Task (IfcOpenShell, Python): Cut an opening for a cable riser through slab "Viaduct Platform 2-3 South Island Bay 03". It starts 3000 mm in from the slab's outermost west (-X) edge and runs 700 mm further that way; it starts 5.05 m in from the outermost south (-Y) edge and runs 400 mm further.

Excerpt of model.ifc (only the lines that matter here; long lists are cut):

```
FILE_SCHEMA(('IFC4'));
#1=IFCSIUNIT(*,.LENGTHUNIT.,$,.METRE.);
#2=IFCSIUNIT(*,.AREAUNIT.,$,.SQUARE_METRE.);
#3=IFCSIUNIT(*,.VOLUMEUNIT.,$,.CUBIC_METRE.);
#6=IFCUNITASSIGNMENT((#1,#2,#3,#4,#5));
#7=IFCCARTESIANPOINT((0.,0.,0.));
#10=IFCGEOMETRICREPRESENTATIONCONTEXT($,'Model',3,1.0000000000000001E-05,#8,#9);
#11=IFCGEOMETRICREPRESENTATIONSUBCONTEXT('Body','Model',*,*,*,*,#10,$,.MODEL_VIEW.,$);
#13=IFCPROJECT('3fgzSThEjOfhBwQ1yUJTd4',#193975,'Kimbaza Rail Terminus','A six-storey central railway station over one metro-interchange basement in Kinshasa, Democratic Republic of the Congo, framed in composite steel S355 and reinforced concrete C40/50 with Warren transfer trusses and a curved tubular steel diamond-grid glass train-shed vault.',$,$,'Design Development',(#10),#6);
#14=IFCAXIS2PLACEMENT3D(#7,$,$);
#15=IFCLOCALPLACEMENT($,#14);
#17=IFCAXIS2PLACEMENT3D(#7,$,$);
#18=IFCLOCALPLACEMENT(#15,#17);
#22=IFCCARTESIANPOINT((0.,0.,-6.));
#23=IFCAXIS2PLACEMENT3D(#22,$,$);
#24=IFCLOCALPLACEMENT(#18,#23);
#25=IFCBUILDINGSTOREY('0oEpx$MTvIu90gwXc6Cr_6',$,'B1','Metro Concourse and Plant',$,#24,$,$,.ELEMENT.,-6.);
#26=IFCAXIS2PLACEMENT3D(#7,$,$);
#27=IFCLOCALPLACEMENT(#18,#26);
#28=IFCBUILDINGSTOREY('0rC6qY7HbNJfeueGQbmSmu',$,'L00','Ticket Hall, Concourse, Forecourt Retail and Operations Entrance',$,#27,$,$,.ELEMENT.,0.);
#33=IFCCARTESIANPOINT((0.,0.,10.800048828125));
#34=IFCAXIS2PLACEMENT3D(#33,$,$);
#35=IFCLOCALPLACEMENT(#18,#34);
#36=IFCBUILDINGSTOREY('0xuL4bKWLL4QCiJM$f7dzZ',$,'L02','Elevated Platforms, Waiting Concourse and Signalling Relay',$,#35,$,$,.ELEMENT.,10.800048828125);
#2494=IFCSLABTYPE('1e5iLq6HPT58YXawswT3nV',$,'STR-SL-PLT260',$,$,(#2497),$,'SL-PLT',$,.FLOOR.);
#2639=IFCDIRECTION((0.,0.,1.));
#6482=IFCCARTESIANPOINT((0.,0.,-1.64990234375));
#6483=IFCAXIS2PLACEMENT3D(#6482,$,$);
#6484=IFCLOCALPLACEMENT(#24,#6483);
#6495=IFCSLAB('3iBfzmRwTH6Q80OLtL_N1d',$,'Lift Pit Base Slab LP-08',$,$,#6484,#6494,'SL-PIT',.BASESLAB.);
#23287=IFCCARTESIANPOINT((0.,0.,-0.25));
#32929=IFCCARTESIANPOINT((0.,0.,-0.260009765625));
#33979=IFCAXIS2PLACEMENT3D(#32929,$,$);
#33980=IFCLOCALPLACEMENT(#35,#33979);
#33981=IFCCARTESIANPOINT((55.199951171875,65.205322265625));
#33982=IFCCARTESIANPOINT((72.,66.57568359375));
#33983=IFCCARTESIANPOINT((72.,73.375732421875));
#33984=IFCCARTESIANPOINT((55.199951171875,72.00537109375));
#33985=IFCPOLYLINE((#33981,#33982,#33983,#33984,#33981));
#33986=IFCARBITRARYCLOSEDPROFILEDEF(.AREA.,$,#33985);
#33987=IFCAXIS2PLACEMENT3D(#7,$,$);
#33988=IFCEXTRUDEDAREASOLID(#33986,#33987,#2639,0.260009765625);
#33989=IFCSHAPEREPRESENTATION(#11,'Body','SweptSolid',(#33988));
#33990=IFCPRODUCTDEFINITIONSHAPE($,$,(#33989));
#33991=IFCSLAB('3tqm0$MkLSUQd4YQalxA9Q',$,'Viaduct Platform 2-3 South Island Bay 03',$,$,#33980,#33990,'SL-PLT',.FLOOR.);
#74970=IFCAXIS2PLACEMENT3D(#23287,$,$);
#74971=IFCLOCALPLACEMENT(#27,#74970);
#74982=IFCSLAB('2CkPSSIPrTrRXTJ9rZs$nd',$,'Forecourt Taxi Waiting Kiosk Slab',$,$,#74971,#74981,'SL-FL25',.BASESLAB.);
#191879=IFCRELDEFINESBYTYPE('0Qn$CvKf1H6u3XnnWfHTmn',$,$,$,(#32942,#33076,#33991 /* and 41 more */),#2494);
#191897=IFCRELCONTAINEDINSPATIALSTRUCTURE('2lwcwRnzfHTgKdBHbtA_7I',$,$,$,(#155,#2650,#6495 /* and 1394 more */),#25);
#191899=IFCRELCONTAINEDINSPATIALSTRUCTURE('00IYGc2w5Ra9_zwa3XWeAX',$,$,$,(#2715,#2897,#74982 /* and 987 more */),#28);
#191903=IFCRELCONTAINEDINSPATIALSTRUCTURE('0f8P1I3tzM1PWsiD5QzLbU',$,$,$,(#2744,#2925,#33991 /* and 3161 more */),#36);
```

```python
import numpy as np
import ifcopenshell
import ifcopenshell.api.feature
import ifcopenshell.api.geometry
import ifcopenshell.api.root
import ifcopenshell.geom
import ifcopenshell.util.placement
import ifcopenshell.util.representation
import ifcopenshell.util.shape
import ifcopenshell.util.unit

model = ifcopenshell.open("model.ifc")
unit_scale = ifcopenshell.util.unit.calculate_unit_scale(model)
settings = ifcopenshell.geom.settings()


def volume(element):
    """Net volume in cubic metres, openings subtracted."""
    shape = ifcopenshell.geom.create_shape(settings, element)
    return ifcopenshell.util.shape.get_volume(shape.geometry)


slab = model.by_guid("3tqm0$MkLSUQd4YQalxA9Q")
before = volume(slab)

# Extent in the slab's own axes, in metres. The edges named are its -X and -Y sides.
slab_shape = ifcopenshell.geom.create_shape(settings, slab)
vertices = ifcopenshell.util.shape.get_vertices(slab_shape.geometry)
x_min, y_min, bottom = vertices.min(axis=0)
top = vertices[:, 2].max()

opening = ifcopenshell.api.root.create_entity(model, ifc_class="IfcOpeningElement", name="Cable riser opening", predefined_type="OPENING")
context = ifcopenshell.util.representation.get_context(model, "Model", "Body", "MODEL_VIEW")
width, depth = 0.7, 0.4
outline = [(0.0, 0.0), (width, 0.0), (width, depth), (0.0, depth), (0.0, 0.0)]
# Overshoot both faces by 50 mm so the cut is clean.
shape = ifcopenshell.api.geometry.add_slab_representation(
    model, context=context, depth=top - bottom + 0.1, polyline=outline
)
ifcopenshell.api.geometry.assign_representation(model, product=opening, representation=shape)

matrix = ifcopenshell.util.placement.get_local_placement(slab.ObjectPlacement)
matrix[:, 3] = matrix @ np.append(np.array([x_min + 3, y_min + 5.05, bottom - 0.05]) / unit_scale, 1.0)
ifcopenshell.api.geometry.edit_object_placement(model, product=opening, matrix=matrix, is_si=False)
ifcopenshell.api.feature.add_feature(model, feature=opening, element=slab)

after = volume(slab)

print(f"slab volume {before:.3f} -> {after:.3f} m3")

model.write("model_v2.ifc")
```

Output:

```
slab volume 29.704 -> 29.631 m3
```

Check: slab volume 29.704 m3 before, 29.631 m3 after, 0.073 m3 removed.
